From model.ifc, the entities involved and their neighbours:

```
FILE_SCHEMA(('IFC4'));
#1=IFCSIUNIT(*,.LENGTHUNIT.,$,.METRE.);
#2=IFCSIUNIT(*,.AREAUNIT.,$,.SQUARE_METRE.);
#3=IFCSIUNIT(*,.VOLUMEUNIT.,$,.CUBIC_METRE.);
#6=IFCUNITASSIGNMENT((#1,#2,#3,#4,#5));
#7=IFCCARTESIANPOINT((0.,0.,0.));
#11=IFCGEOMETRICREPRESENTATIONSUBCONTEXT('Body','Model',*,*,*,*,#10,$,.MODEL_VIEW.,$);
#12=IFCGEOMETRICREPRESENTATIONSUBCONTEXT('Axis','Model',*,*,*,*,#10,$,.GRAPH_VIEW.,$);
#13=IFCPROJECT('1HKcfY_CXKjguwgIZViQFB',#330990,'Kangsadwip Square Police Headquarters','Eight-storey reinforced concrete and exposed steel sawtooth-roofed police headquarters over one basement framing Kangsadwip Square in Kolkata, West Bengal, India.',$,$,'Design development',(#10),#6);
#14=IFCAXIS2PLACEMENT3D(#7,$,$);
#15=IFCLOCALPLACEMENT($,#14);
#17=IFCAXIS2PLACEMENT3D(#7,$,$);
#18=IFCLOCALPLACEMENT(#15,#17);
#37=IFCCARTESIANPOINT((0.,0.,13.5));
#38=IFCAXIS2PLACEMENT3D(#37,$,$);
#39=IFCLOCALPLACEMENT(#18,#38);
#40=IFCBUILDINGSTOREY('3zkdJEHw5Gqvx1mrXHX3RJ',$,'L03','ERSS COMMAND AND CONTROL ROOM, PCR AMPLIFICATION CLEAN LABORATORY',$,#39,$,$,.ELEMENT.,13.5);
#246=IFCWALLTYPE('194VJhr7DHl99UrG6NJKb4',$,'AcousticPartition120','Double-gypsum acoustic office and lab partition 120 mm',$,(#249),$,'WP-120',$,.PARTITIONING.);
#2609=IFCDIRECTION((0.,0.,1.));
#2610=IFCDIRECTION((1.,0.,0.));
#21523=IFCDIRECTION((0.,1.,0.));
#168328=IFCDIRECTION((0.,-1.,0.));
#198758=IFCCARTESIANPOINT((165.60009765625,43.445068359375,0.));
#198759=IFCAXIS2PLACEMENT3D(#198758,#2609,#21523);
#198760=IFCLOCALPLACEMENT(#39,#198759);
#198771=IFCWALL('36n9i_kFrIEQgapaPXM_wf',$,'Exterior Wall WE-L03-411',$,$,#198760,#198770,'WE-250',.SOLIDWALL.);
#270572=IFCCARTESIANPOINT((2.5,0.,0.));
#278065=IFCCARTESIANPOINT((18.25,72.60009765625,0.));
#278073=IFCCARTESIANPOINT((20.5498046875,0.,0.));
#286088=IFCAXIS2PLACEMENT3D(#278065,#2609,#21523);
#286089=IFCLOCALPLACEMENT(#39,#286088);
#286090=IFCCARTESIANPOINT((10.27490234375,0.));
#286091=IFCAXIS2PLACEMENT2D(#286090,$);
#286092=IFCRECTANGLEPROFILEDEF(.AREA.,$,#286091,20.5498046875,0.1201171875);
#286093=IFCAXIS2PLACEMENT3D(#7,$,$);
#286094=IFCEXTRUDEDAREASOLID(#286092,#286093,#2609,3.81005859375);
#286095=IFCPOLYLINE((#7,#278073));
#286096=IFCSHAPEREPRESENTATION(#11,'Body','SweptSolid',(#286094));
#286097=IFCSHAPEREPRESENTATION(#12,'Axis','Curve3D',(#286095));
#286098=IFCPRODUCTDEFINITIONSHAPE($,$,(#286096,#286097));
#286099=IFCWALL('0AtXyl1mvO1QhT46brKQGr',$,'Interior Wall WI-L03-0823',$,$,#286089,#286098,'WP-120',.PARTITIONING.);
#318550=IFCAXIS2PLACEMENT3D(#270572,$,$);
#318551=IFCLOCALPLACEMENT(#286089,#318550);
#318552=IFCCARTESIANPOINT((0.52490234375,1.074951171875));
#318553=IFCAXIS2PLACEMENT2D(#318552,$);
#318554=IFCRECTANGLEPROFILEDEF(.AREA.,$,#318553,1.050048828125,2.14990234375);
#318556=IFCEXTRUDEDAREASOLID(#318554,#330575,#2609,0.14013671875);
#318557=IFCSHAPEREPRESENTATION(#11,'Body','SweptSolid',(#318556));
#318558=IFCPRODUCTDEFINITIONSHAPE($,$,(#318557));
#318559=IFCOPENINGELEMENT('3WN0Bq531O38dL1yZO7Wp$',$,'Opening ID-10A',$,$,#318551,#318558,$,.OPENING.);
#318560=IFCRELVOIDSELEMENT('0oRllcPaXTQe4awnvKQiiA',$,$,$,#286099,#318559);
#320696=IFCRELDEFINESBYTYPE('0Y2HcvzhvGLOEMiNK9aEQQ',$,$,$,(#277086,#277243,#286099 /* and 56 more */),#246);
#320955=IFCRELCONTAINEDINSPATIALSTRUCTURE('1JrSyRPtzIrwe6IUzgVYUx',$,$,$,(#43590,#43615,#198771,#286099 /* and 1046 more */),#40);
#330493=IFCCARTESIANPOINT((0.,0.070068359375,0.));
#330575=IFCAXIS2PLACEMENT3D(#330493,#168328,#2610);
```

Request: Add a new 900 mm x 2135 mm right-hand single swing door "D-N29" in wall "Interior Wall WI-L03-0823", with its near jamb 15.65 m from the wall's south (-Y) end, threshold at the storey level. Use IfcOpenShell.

```python
import numpy as np
import ifcopenshell
import ifcopenshell.api.feature
import ifcopenshell.api.geometry
import ifcopenshell.api.root
import ifcopenshell.api.spatial
import ifcopenshell.geom
import ifcopenshell.util.element
import ifcopenshell.util.placement
import ifcopenshell.util.representation
import ifcopenshell.util.shape
import ifcopenshell.util.unit

model = ifcopenshell.open("model.ifc")
unit_scale = ifcopenshell.util.unit.calculate_unit_scale(model)
settings = ifcopenshell.geom.settings()


def volume(element):
    """Net volume in cubic metres, openings subtracted."""
    shape = ifcopenshell.geom.create_shape(settings, element)
    return ifcopenshell.util.shape.get_volume(shape.geometry)


wall = model.by_guid("0AtXyl1mvO1QhT46brKQGr")
storey = ifcopenshell.util.element.get_container(wall, ifc_class="IfcBuildingStorey")
context = ifcopenshell.util.representation.get_context(model, "Model", "Body", "MODEL_VIEW")
before = volume(wall)

width, height, from_end, sill = 0.9, 2.135, 15.65, 0.0  # metres

# The wall runs along its own X axis, and the end named is its -X end.
wall_shape = ifcopenshell.geom.create_shape(settings, wall)
x, y, z = ifcopenshell.util.shape.get_vertices(wall_shape.geometry).T
start = x.min() + from_end
face, thickness = float(y.min()), float(y.max() - y.min())
wall_matrix = ifcopenshell.util.placement.get_local_placement(wall.ObjectPlacement)
level = ifcopenshell.util.placement.get_local_placement(storey.ObjectPlacement)[2, 3]


def in_wall(x, y):
    """Placement at x, y metres in the wall's axes, at sill height."""
    matrix = wall_matrix.copy()
    matrix[:, 3] = wall_matrix @ np.array([x / unit_scale, y / unit_scale, 0.0, 1.0])
    matrix[2, 3] = level + sill / unit_scale
    return matrix


# Opening: a box that overshoots both wall faces by 50 mm.
opening = ifcopenshell.api.root.create_entity(model, ifc_class="IfcOpeningElement", predefined_type="OPENING")
box = ifcopenshell.api.geometry.add_wall_representation(
    model, context=context, length=width, height=height, thickness=thickness + 0.1
)
ifcopenshell.api.geometry.assign_representation(model, product=opening, representation=box)
ifcopenshell.api.geometry.edit_object_placement(model, product=opening, matrix=in_wall(start, face - 0.05), is_si=False)
ifcopenshell.api.feature.add_feature(model, feature=opening, element=wall)

door = ifcopenshell.api.root.create_entity(model, ifc_class="IfcDoor", name="D-N29", predefined_type="DOOR")
door.OverallWidth, door.OverallHeight = width / unit_scale, height / unit_scale
door.OperationType = "SINGLE_SWING_RIGHT"
body = ifcopenshell.api.geometry.add_door_representation(
    model,
    context=context,
    overall_width=door.OverallWidth,
    overall_height=door.OverallHeight,
    operation_type="SINGLE_SWING_RIGHT",
    lining_properties={"LiningDepth": thickness / unit_scale, "ThresholdDepth": thickness / unit_scale},
)
ifcopenshell.api.geometry.assign_representation(model, product=door, representation=body)
ifcopenshell.api.spatial.assign_container(model, products=[door], relating_structure=storey)
ifcopenshell.api.feature.add_filling(model, opening=opening, element=door)

# The lining spans the wall, so the door starts at the wall face.
ifcopenshell.api.geometry.edit_object_placement(model, product=door, matrix=in_wall(start, face), is_si=False)

after = volume(wall)

print(f"wall volume {before:.3f} -> {after:.3f} m3")

model.write("model_edited.ifc")
```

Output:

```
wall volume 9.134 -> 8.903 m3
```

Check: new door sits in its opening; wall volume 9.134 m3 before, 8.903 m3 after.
